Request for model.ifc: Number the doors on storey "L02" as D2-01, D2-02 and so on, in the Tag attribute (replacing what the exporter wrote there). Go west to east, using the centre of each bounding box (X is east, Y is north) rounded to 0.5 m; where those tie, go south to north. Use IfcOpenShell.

First a look at what the model holds.

```python
import ifcopenshell
import ifcopenshell.util.element
import ifcopenshell.util.placement

model = ifcopenshell.open("model.ifc")
print(model.schema)
storey = next(s for s in model.by_type("IfcBuildingStorey") if s.Name == "L02")
doors = [e for e in ifcopenshell.util.element.get_decomposition(storey) if e.is_a("IfcDoor")]
for e in sorted(doors, key=lambda e: e.id()):
    origin = ifcopenshell.util.placement.get_local_placement(e.ObjectPlacement)[:3, 3]
    print(e.id(), e.Tag, e.Name, origin.round(2) + 0.0, sep=" | ")
```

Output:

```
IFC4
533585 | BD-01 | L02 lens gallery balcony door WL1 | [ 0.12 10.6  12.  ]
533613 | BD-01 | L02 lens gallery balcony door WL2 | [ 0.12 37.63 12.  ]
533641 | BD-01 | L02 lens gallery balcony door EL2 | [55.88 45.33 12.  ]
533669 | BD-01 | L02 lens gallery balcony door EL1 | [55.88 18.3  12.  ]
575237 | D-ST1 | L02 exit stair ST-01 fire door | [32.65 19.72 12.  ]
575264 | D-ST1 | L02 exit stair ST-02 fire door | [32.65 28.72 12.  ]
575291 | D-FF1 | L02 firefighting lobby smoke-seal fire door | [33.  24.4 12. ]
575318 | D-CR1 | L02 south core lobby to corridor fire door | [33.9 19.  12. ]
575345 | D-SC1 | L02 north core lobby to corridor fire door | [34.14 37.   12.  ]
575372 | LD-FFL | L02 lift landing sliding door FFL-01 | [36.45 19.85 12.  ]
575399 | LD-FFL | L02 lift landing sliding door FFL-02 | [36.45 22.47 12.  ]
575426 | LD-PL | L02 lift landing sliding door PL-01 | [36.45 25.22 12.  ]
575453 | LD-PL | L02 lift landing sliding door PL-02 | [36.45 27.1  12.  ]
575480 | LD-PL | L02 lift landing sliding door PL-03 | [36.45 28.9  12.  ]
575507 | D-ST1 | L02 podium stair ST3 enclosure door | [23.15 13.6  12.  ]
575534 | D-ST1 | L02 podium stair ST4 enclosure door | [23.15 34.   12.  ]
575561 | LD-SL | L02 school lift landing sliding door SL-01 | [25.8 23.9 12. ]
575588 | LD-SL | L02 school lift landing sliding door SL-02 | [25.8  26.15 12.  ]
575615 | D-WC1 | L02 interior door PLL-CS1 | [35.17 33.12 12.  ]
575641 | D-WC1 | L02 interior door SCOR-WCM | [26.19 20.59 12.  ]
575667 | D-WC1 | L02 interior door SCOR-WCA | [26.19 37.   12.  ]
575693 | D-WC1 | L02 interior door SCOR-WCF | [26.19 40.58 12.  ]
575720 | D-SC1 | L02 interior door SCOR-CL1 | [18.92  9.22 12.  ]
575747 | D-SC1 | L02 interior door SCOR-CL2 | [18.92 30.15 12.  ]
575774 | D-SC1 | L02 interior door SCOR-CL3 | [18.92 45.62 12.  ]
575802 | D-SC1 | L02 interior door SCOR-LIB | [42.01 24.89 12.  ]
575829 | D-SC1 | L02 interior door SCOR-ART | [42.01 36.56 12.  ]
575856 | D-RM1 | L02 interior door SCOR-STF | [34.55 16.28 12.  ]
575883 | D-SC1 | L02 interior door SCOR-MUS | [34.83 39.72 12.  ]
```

```python
import ifcopenshell
import ifcopenshell.geom
import ifcopenshell.util.element
import ifcopenshell.util.shape

model = ifcopenshell.open("model.ifc")
settings = ifcopenshell.geom.settings()
settings.set("use-world-coords", True)


def centre(element):
    shape = ifcopenshell.geom.create_shape(settings, element)
    return ifcopenshell.util.shape.get_bbox_centroid(shape.geometry)


storey = next(s for s in model.by_type("IfcBuildingStorey") if s.Name == "L02")
doors = [e for e in ifcopenshell.util.element.get_decomposition(storey) if e.is_a("IfcDoor")]

# Insertion points can sit at a corner or the storey origin, so sort by the geometry (in metres).
centres = {e: centre(e) for e in doors}
doors.sort(key=lambda e: (round(centres[e][0] / 0.5), centres[e][1]))

for i, e in enumerate(doors, start=1):
    number = f"D2-{i:02d}"
    e.Tag = number
    print(e.id(), number)

model.write("model-out.ifc")
```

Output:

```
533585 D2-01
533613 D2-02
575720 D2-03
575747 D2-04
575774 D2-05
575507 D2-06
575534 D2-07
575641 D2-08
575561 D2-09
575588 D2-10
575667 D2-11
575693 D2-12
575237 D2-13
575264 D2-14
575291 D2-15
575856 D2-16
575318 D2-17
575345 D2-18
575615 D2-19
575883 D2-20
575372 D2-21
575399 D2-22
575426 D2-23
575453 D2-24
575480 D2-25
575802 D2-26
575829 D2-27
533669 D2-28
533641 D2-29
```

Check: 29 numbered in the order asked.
